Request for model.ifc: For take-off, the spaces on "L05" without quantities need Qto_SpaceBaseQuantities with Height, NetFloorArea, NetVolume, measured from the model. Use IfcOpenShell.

First a look at what the model holds.

```python
import ifcopenshell
import ifcopenshell.util.element
import ifcopenshell.util.unit

model = ifcopenshell.open("model.ifc")
print(model.schema)
for unit_type in ("LENGTHUNIT", "AREAUNIT", "VOLUMEUNIT"):
    print(unit_type, ifcopenshell.util.unit.calculate_unit_scale(model, unit_type))
storey = next(s for s in model.by_type("IfcBuildingStorey") if s.Name == "L05")
spaces = [e for e in ifcopenshell.util.element.get_decomposition(storey) if e.is_a("IfcSpace")]
for e in sorted(spaces, key=lambda e: e.id()):
    print(e.id(), e.is_a(), e.Name, list(ifcopenshell.util.element.get_psets(e, qtos_only=True)), sep=" | ")
```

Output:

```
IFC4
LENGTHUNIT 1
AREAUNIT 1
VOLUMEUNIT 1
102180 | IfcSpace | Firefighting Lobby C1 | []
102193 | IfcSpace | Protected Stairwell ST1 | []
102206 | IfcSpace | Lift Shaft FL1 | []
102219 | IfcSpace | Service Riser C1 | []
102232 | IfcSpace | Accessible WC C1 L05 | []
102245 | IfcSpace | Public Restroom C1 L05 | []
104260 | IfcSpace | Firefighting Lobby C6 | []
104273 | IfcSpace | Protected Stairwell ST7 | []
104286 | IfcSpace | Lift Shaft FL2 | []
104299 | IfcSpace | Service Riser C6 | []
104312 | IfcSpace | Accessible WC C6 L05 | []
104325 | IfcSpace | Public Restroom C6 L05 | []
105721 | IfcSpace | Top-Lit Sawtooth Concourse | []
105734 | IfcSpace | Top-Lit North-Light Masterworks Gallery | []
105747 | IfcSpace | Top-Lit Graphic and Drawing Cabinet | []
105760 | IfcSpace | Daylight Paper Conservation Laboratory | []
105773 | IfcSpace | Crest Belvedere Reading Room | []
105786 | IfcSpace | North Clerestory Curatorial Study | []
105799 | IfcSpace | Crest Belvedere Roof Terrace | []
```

```python
import ifcopenshell
import ifcopenshell.api.pset
import ifcopenshell.geom
import ifcopenshell.util.element
import ifcopenshell.util.shape
import ifcopenshell.util.unit

model = ifcopenshell.open("model.ifc")
unit_scale = ifcopenshell.util.unit.calculate_unit_scale(model)
area_scale = ifcopenshell.util.unit.calculate_unit_scale(model, "AREAUNIT")
volume_scale = ifcopenshell.util.unit.calculate_unit_scale(model, "VOLUMEUNIT")
settings = ifcopenshell.geom.settings()

storey = next(s for s in model.by_type("IfcBuildingStorey") if s.Name == "L05")
spaces = [e for e in ifcopenshell.util.element.get_decomposition(storey) if e.is_a("IfcSpace")]

for e in sorted(spaces, key=lambda e: e.id()):
    if ifcopenshell.util.element.get_psets(e, qtos_only=True, should_inherit=False):
        continue
    # Geometry comes back in metres, in the element's own axes.
    shape = ifcopenshell.geom.create_shape(settings, e)
    values = {
        "Height": ifcopenshell.util.shape.get_z(shape.geometry) / unit_scale,
        "NetFloorArea": ifcopenshell.util.shape.get_footprint_area(shape.geometry) / area_scale,
        "NetVolume": ifcopenshell.util.shape.get_volume(shape.geometry) / volume_scale,
    }
    qto = ifcopenshell.api.pset.add_qto(model, product=e, name="Qto_SpaceBaseQuantities")
    ifcopenshell.api.pset.edit_qto(model, qto=qto, properties=values)
    print(e.id(), {k: round(v, 3) for k, v in values.items()})

model.write("model_rev.ifc")
```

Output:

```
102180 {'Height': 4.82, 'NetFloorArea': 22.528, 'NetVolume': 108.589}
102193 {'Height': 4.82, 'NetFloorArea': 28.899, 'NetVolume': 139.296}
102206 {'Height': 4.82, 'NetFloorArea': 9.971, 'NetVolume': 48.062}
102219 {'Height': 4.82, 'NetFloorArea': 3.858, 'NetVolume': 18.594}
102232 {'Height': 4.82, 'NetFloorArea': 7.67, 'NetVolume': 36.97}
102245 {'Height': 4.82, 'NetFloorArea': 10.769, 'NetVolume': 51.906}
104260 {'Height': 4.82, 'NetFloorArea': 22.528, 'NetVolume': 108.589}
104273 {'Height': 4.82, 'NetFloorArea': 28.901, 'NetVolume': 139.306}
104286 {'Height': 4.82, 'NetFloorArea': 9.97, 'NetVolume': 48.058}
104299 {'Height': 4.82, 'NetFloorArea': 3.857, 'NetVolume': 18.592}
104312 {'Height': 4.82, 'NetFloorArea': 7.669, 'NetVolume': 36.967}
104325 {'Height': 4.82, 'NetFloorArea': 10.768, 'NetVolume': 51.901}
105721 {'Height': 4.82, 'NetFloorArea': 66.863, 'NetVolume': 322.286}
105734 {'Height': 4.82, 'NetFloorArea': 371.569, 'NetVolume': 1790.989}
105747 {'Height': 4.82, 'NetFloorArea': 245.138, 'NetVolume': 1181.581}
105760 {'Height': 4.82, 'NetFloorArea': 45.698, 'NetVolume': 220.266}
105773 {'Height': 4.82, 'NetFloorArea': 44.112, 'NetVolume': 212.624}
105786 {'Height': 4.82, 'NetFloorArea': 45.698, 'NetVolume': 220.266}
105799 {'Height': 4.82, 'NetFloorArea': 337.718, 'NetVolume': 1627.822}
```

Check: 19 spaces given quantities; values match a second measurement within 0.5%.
